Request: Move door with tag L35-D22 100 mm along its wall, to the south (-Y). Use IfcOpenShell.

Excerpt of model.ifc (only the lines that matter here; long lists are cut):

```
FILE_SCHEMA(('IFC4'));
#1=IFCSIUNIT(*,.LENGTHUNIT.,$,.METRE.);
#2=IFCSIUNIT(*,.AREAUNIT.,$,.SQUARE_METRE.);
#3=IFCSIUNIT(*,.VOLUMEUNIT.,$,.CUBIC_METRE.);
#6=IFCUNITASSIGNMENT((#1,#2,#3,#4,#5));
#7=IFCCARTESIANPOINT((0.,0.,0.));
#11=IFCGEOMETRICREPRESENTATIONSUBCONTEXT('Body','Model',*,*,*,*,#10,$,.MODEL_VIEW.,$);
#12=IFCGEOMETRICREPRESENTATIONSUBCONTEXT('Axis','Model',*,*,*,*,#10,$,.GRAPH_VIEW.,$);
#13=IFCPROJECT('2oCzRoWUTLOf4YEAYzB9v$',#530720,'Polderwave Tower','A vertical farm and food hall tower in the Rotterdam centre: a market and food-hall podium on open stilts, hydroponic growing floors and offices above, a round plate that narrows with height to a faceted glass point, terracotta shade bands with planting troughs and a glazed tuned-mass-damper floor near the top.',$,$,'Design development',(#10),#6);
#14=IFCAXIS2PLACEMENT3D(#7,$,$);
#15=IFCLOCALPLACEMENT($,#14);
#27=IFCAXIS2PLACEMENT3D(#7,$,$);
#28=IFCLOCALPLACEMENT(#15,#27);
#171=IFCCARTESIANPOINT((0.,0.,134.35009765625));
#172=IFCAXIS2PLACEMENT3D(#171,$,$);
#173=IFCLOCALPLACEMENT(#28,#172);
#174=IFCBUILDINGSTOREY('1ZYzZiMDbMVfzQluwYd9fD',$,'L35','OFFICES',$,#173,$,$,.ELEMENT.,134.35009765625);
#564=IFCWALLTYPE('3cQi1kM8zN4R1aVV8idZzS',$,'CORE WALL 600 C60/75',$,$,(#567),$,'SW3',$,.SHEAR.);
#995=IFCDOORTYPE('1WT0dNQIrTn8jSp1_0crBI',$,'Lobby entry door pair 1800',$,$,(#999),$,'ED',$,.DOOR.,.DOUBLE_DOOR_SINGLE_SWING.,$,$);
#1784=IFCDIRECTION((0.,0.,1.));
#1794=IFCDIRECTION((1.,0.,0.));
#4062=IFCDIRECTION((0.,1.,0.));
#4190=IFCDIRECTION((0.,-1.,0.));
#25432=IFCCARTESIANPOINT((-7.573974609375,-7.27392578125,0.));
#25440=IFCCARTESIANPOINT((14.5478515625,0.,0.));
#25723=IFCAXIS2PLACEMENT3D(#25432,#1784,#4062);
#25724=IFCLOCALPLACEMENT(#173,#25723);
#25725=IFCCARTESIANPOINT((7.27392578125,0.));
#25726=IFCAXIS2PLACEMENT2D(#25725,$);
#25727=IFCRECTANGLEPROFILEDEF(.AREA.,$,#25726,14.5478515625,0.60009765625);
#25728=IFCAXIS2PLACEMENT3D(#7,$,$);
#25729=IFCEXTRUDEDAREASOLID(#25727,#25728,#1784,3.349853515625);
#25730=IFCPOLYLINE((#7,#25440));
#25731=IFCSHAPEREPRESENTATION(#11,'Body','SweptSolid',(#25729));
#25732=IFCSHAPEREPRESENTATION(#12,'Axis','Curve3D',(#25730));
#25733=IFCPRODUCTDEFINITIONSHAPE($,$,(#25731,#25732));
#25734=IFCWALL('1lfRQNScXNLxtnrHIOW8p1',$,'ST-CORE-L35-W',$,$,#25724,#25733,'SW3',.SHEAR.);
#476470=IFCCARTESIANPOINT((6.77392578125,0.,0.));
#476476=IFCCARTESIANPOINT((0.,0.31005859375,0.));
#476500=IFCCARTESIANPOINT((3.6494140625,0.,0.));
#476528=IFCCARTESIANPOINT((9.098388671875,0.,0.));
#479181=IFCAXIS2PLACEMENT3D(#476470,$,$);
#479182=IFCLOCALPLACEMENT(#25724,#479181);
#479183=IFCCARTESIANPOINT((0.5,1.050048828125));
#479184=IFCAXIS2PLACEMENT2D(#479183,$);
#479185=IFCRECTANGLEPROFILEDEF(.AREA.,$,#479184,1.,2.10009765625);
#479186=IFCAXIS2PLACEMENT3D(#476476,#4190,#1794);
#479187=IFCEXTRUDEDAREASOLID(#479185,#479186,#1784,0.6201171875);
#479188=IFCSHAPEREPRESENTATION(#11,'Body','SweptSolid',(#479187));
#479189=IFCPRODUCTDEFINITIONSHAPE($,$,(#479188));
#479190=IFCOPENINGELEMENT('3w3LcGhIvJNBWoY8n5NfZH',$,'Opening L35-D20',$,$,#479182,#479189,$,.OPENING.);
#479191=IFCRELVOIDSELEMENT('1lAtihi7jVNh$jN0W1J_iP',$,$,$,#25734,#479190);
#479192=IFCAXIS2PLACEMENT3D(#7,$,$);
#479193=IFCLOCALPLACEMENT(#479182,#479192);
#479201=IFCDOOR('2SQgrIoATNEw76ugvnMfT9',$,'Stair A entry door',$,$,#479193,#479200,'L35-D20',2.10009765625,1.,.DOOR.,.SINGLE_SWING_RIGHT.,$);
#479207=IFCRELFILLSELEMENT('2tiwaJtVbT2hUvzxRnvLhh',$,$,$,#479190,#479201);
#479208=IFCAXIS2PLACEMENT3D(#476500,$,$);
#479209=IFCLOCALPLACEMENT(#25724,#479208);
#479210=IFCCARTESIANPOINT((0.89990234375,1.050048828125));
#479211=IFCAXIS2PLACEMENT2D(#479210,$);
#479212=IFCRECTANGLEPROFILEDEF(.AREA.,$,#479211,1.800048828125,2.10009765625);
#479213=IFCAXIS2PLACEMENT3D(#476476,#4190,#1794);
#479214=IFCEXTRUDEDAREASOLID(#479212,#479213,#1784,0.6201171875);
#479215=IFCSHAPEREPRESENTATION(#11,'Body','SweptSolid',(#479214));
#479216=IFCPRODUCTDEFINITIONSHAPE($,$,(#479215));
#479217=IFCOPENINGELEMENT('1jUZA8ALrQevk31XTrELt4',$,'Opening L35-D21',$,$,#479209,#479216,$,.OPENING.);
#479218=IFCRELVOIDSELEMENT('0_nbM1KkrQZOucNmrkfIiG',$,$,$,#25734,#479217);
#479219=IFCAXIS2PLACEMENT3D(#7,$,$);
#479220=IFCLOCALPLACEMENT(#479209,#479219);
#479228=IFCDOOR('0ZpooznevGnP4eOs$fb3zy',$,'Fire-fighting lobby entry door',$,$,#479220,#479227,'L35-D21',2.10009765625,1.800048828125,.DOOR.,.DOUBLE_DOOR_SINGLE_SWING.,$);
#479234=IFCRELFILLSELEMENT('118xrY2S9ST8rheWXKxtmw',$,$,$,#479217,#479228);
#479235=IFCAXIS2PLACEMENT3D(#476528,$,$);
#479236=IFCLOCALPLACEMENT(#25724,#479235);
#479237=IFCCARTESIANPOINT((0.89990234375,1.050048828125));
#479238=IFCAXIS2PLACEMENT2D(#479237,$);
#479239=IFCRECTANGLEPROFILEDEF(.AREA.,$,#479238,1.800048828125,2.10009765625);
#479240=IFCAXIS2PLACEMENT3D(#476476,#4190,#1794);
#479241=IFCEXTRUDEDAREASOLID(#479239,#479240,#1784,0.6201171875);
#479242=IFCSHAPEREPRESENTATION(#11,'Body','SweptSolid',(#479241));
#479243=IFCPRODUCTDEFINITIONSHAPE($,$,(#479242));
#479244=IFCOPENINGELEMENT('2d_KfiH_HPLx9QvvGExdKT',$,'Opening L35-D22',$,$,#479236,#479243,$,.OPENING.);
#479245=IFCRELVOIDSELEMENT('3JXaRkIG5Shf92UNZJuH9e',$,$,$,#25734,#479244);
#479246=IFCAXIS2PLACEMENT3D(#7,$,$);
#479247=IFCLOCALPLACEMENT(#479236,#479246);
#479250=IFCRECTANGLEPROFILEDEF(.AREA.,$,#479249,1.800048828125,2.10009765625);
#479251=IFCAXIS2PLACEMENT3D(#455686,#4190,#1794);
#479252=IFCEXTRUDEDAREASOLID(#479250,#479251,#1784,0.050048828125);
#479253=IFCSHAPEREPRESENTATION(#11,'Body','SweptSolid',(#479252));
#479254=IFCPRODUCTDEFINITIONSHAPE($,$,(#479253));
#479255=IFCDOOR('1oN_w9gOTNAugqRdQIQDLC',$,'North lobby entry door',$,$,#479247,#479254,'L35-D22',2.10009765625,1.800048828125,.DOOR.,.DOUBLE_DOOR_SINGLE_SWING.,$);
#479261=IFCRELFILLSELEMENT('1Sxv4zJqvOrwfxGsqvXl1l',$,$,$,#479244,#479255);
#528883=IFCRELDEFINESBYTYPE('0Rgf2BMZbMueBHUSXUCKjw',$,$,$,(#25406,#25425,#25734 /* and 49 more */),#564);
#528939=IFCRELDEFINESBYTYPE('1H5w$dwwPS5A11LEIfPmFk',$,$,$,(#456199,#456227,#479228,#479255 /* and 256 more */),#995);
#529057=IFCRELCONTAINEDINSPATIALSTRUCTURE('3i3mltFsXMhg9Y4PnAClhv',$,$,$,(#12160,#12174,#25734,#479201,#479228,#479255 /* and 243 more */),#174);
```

```python
import ifcopenshell
import ifcopenshell.api.geometry
import ifcopenshell.util.placement

model = ifcopenshell.open("model.ifc")

door = model.by_guid("1oN_w9gOTNAugqRdQIQDLC")
opening = door.FillsVoids[0].RelatingOpeningElement
wall = opening.VoidsElements[0].RelatingBuildingElement

wall_matrix = ifcopenshell.util.placement.get_local_placement(wall.ObjectPlacement)
shift = wall_matrix[:3, 0] * -0.1
before = ifcopenshell.util.placement.get_local_placement(door.ObjectPlacement)[:3, 3].copy()

# The door is placed relative to its opening, so it follows when the opening moves.
matrix = ifcopenshell.util.placement.get_local_placement(opening.ObjectPlacement)
matrix[:3, 3] += shift
ifcopenshell.api.geometry.edit_object_placement(
    model, product=opening, matrix=matrix, is_si=False, should_transform_children=True
)

after = ifcopenshell.util.placement.get_local_placement(door.ObjectPlacement)[:3, 3]
print("door moved by", (after - before).round(3) + 0.0)

model.write("model_edited.ifc")
```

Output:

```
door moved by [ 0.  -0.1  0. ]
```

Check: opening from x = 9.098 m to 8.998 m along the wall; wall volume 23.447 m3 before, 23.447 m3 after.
